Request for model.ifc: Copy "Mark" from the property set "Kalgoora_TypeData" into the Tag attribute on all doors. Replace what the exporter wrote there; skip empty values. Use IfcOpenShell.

First a look at what the model holds.

```python
import ifcopenshell
import ifcopenshell.util.element

model = ifcopenshell.open("model.ifc")
print(model.schema)
doors = model.by_type("IfcDoor")
print(len(doors), "doors")
for e in doors[:8]:
    source = ifcopenshell.util.element.get_pset(e, "Kalgoora_TypeData", "Mark")
    target = e.Tag
    print(e.id(), repr(source), repr(target), sep=" | ")
```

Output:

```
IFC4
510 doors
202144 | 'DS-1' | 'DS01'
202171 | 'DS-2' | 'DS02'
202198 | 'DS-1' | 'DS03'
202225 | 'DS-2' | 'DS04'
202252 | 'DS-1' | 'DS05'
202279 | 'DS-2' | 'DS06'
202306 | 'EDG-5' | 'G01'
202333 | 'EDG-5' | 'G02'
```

```python
import ifcopenshell
import ifcopenshell.util.element

model = ifcopenshell.open("model.ifc")

count = 0
for e in model.by_type("IfcDoor"):
    value = ifcopenshell.util.element.get_pset(e, "Kalgoora_TypeData", "Mark")
    current = e.Tag
    if not value or not value.strip() or current == value:
        continue
    e.Tag = value
    count += 1

print(count, "doors updated")

model.write("model_v2.ifc")
```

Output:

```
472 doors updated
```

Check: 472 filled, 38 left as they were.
